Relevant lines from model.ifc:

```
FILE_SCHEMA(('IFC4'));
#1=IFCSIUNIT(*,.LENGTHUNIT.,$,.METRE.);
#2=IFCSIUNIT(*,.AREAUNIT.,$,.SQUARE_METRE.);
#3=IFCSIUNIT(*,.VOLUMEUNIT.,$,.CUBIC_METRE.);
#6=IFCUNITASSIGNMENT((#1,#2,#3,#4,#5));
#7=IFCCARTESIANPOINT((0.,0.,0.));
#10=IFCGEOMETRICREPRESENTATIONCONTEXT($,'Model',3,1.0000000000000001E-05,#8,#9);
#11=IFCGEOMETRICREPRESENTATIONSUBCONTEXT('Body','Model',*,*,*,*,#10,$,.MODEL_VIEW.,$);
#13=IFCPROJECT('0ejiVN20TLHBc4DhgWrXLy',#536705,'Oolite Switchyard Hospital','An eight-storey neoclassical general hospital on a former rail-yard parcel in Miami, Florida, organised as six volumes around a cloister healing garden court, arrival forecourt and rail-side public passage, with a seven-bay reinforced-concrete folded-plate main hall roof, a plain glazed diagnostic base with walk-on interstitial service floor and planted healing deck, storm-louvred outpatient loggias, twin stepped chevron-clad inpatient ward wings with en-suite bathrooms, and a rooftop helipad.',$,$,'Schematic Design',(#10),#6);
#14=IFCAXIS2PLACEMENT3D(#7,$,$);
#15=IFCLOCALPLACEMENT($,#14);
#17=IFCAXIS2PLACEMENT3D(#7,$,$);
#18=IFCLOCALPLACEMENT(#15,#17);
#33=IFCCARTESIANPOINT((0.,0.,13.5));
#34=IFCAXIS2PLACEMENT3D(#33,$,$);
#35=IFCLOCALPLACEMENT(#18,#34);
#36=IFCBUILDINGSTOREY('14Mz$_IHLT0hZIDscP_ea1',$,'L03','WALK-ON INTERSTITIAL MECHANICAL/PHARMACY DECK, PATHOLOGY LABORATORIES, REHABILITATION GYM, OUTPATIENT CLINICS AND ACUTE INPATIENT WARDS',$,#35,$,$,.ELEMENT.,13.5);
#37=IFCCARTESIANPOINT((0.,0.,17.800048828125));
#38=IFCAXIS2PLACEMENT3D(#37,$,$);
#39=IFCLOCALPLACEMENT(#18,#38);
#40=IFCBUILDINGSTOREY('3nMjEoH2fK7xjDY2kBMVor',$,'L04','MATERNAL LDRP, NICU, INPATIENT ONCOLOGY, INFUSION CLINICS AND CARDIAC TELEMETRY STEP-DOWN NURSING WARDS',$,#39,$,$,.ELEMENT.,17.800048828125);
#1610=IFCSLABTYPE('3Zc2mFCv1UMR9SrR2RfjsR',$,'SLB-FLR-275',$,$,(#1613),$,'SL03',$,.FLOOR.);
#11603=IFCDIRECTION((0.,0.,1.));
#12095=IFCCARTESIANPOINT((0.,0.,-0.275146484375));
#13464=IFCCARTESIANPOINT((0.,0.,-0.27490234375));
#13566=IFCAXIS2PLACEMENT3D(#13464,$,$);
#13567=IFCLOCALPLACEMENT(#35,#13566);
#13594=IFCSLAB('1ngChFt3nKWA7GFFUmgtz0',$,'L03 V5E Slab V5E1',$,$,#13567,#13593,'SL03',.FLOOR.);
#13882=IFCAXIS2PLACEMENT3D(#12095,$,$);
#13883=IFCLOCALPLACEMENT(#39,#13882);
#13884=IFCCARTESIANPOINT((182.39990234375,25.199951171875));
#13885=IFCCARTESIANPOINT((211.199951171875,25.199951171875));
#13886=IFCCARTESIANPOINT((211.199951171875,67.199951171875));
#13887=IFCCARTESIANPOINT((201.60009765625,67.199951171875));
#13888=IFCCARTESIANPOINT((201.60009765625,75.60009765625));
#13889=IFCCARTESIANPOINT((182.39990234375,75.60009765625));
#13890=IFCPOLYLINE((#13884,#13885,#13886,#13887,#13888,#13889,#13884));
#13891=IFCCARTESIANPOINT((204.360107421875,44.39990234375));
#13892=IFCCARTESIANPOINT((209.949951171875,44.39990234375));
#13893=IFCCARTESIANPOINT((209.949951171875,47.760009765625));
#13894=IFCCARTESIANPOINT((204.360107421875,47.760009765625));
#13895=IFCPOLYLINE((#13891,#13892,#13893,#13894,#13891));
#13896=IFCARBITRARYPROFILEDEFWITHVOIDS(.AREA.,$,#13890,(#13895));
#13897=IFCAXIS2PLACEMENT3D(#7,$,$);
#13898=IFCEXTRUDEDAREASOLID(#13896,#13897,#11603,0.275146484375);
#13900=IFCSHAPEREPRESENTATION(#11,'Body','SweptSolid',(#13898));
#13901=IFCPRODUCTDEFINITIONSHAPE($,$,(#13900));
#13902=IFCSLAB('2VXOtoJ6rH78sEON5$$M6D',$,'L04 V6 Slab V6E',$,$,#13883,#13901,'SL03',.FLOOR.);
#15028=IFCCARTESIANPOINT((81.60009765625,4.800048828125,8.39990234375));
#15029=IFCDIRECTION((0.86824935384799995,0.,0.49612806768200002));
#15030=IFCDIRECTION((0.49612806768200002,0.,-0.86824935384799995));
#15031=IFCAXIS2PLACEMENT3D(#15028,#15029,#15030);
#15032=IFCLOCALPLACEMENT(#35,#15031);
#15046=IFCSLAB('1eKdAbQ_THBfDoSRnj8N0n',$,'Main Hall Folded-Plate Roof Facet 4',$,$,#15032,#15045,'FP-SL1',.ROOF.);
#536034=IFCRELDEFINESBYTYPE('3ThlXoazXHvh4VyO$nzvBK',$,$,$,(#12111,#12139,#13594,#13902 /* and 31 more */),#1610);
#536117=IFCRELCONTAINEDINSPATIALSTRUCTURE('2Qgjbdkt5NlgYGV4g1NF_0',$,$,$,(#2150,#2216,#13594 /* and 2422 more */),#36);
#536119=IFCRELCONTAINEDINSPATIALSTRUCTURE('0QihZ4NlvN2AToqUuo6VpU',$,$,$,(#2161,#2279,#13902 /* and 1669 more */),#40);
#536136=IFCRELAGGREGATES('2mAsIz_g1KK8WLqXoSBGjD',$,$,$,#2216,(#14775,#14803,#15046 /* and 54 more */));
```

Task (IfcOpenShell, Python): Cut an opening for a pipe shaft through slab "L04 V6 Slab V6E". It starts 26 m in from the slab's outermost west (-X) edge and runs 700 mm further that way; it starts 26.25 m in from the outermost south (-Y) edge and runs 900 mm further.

```python
import numpy as np
import ifcopenshell
import ifcopenshell.api.feature
import ifcopenshell.api.geometry
import ifcopenshell.api.root
import ifcopenshell.geom
import ifcopenshell.util.placement
import ifcopenshell.util.representation
import ifcopenshell.util.shape
import ifcopenshell.util.unit

model = ifcopenshell.open("model.ifc")
unit_scale = ifcopenshell.util.unit.calculate_unit_scale(model)
settings = ifcopenshell.geom.settings()


def volume(element):
    """Net volume in cubic metres, openings subtracted."""
    shape = ifcopenshell.geom.create_shape(settings, element)
    return ifcopenshell.util.shape.get_volume(shape.geometry)


slab = model.by_guid("2VXOtoJ6rH78sEON5$$M6D")
before = volume(slab)

# Extent in the slab's own axes, in metres. The edges named are its -X and -Y sides.
slab_shape = ifcopenshell.geom.create_shape(settings, slab)
vertices = ifcopenshell.util.shape.get_vertices(slab_shape.geometry)
x_min, y_min, bottom = vertices.min(axis=0)
top = vertices[:, 2].max()

opening = ifcopenshell.api.root.create_entity(model, ifc_class="IfcOpeningElement", name="Pipe shaft opening", predefined_type="OPENING")
context = ifcopenshell.util.representation.get_context(model, "Model", "Body", "MODEL_VIEW")
width, depth = 0.7, 0.9
outline = [(0.0, 0.0), (width, 0.0), (width, depth), (0.0, depth), (0.0, 0.0)]
# Overshoot both faces by 50 mm so the cut is clean.
shape = ifcopenshell.api.geometry.add_slab_representation(
    model, context=context, depth=top - bottom + 0.1, polyline=outline
)
ifcopenshell.api.geometry.assign_representation(model, product=opening, representation=shape)

matrix = ifcopenshell.util.placement.get_local_placement(slab.ObjectPlacement)
matrix[:, 3] = matrix @ np.append(np.array([x_min + 26, y_min + 26.25, bottom - 0.05]) / unit_scale, 1.0)
ifcopenshell.api.geometry.edit_object_placement(model, product=opening, matrix=matrix, is_si=False)
ifcopenshell.api.feature.add_feature(model, feature=opening, element=slab)

after = volume(slab)

print(f"slab volume {before:.3f} -> {after:.3f} m3")

model.write("model_edited.ifc")
```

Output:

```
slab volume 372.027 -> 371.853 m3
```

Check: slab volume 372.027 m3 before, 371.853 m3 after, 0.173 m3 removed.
